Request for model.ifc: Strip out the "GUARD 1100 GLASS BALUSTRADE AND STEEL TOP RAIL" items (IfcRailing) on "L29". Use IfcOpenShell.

First a look at what the model holds.

```python
import ifcopenshell
import ifcopenshell.util.element

model = ifcopenshell.open("model.ifc")
print(model.schema)
storey = next(s for s in model.by_type("IfcBuildingStorey") if s.Name == "L29")
railings = [e for e in ifcopenshell.util.element.get_decomposition(storey) if e.is_a("IfcRailing")]
seen = {}
for e in railings:
    element_type = ifcopenshell.util.element.get_type(e)
    name = element_type.Name if element_type not in (None, e) else None
    seen[name] = seen.get(name, 0) + 1
for name, count in sorted(seen.items(), key=str):
    print(count, "x", name)
```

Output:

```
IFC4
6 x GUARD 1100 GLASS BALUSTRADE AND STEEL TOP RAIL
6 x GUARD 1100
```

```python
import ifcopenshell
import ifcopenshell.api.root
import ifcopenshell.util.element

model = ifcopenshell.open("model.ifc")

storey = next(s for s in model.by_type("IfcBuildingStorey") if s.Name == "L29")
railings = [e for e in ifcopenshell.util.element.get_decomposition(storey) if e.is_a("IfcRailing")]
targets = [e for e in railings if (t := ifcopenshell.util.element.get_type(e)) not in (None, e) and t.Name == "GUARD 1100 GLASS BALUSTRADE AND STEEL TOP RAIL"]

for e in targets:
    ifcopenshell.api.root.remove_product(model, product=e)
print(len(targets), "removed")

model.write("model_rev.ifc")
```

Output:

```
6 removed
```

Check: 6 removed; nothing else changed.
